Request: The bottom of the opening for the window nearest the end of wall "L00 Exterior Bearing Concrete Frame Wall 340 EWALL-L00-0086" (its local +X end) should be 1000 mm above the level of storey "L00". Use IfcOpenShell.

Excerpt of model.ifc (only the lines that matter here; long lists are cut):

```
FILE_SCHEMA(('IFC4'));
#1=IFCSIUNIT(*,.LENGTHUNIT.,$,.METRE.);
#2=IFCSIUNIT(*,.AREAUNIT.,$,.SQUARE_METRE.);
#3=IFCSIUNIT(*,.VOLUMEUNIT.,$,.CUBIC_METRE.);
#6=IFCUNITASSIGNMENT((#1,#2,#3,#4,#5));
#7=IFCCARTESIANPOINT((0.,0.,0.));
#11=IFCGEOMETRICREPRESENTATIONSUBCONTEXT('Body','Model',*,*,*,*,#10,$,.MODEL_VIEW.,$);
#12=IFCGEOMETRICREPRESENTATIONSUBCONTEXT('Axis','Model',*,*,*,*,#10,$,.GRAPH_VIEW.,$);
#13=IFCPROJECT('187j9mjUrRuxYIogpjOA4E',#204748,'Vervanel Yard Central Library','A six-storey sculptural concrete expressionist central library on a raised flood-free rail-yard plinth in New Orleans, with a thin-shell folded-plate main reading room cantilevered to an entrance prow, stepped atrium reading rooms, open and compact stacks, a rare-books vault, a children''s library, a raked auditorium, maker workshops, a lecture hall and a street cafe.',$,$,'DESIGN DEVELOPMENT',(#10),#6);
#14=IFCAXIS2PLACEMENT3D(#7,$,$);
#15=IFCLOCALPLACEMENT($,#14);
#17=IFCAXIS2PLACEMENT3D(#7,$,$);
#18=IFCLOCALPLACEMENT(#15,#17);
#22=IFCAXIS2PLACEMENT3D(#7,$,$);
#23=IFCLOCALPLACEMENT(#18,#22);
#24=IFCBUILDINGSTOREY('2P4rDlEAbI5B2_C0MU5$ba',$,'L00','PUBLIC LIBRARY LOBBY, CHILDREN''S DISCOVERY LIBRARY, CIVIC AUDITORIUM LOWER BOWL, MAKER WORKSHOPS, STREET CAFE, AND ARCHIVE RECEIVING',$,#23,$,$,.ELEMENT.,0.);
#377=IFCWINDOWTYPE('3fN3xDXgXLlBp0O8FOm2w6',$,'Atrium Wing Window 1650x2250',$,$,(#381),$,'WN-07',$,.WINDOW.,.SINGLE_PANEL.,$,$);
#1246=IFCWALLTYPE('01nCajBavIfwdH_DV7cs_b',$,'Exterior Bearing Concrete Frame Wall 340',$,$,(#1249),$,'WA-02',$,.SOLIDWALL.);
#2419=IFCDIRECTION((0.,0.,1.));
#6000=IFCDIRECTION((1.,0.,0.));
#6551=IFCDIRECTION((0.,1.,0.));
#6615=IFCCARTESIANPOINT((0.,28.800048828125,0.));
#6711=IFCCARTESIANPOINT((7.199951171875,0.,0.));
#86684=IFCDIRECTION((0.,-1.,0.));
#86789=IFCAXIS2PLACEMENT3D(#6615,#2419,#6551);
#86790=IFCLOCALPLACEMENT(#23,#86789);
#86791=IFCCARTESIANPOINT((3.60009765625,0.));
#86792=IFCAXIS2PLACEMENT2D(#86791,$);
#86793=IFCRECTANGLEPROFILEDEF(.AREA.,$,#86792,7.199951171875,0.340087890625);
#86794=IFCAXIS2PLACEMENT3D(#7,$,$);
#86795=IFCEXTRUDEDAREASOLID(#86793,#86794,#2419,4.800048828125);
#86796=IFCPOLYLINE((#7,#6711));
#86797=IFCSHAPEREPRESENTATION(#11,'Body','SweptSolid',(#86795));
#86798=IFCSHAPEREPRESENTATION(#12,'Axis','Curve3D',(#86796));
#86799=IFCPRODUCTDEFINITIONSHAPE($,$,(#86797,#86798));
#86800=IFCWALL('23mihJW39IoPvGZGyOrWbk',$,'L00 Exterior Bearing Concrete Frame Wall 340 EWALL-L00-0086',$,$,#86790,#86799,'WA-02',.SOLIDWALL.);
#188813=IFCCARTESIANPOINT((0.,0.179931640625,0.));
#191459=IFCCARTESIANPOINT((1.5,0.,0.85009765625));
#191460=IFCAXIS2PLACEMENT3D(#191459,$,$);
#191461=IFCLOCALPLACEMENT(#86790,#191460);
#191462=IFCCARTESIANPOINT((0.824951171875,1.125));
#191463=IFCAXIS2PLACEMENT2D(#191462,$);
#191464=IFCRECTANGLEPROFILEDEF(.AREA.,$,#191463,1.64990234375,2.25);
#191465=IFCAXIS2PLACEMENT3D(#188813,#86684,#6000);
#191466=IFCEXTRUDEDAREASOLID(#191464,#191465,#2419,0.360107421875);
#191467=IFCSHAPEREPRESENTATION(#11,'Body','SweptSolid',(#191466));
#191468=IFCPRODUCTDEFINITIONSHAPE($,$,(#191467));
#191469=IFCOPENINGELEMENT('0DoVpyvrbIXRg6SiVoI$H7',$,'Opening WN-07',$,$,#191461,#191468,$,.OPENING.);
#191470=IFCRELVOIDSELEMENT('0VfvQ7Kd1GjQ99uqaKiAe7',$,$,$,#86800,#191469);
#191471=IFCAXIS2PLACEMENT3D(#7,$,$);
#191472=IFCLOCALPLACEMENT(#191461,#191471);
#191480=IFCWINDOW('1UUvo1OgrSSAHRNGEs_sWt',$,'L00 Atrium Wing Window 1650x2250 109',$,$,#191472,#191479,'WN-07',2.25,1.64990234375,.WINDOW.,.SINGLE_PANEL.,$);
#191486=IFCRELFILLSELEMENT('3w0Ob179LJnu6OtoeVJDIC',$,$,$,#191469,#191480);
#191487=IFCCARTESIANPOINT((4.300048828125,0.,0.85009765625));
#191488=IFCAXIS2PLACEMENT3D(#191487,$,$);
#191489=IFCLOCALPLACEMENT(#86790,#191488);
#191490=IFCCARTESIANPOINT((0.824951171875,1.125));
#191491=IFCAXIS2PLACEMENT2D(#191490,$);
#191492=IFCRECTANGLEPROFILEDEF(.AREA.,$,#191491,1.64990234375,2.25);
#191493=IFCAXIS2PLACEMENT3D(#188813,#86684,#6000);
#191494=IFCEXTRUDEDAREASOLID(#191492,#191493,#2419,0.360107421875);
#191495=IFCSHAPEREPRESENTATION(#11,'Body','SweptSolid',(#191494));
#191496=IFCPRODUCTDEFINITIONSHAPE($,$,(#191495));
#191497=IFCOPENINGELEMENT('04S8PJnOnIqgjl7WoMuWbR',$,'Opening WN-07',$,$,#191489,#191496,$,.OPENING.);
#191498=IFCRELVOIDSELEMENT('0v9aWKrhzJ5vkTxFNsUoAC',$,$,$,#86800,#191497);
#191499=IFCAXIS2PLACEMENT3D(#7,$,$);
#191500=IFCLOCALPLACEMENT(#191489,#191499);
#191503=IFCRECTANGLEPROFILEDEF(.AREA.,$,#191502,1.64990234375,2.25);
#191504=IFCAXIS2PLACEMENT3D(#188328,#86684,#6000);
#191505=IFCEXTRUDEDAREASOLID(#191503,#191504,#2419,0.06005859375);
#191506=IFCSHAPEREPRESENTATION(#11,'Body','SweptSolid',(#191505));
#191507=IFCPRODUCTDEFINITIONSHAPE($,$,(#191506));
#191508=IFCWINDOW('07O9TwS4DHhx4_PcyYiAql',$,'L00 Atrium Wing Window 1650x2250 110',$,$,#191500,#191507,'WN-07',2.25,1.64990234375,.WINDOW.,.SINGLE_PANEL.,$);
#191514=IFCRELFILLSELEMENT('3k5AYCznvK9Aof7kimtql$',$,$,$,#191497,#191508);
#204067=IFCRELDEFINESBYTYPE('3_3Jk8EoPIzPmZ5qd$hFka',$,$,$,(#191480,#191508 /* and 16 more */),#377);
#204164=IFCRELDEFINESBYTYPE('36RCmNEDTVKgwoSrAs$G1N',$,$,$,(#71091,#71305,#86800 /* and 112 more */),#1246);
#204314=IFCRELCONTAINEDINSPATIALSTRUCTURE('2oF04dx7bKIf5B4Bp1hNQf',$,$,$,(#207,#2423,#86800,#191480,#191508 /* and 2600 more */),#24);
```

```python
import numpy as np
import ifcopenshell
import ifcopenshell.api.geometry
import ifcopenshell.geom
import ifcopenshell.util.element
import ifcopenshell.util.placement
import ifcopenshell.util.shape
import ifcopenshell.util.unit

model = ifcopenshell.open("model.ifc")
unit_scale = ifcopenshell.util.unit.calculate_unit_scale(model)

window = model.by_guid("07O9TwS4DHhx4_PcyYiAql")
opening = window.FillsVoids[0].RelatingOpeningElement
storey = ifcopenshell.util.element.get_container(window, ifc_class="IfcBuildingStorey")
level = ifcopenshell.util.placement.get_local_placement(storey.ObjectPlacement)[2, 3]

# The opening's origin need not be at the sill, so measure its lowest point.
shape = ifcopenshell.geom.create_shape(ifcopenshell.geom.settings(), opening)
bottom = ifcopenshell.util.shape.get_shape_bottom_elevation(shape, shape.geometry) / unit_scale
dz = level + 1 / unit_scale - bottom

shift = np.array([0.0, 0.0, dz])
# The window is placed relative to its opening, so it follows when the opening moves.
matrix = ifcopenshell.util.placement.get_local_placement(opening.ObjectPlacement)
matrix[:3, 3] += shift
ifcopenshell.api.geometry.edit_object_placement(
    model, product=opening, matrix=matrix, is_si=False, should_transform_children=True
)

print(f"moved by {dz * unit_scale:+.3f} m")

model.write("model_updated.ifc")
```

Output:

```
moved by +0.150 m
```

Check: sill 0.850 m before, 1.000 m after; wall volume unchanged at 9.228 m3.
